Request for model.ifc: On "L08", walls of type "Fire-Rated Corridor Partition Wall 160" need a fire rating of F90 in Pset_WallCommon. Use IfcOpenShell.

First a look at what the model holds.

```python
import ifcopenshell
import ifcopenshell.util.element

model = ifcopenshell.open("model.ifc")
print(model.schema)
storey = next(s for s in model.by_type("IfcBuildingStorey") if s.Name == "L08")
walls = [e for e in ifcopenshell.util.element.get_decomposition(storey) if e.is_a("IfcWall")]
seen = {}
for e in walls:
    element_type = ifcopenshell.util.element.get_type(e)
    key = (element_type.Name if element_type != e and element_type else None, ifcopenshell.util.element.get_pset(e, "Pset_WallCommon", "FireRating"))
    seen[key] = seen.get(key, 0) + 1
for (name, value), count in sorted(seen.items(), key=str):
    print(count, "x", name, "|", value)
```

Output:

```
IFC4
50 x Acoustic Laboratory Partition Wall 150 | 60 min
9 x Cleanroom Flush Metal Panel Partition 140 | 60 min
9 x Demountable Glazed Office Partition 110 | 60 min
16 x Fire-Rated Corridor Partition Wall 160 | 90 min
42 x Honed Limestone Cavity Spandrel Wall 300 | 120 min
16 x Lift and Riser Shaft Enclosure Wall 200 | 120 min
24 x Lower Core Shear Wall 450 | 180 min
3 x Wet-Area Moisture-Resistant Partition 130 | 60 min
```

```python
import ifcopenshell
import ifcopenshell.api.pset
import ifcopenshell.util.element

model = ifcopenshell.open("model.ifc")

storey = next(s for s in model.by_type("IfcBuildingStorey") if s.Name == "L08")
walls = [e for e in ifcopenshell.util.element.get_decomposition(storey) if e.is_a("IfcWall")]

count = 0
for e in walls:
    element_type = ifcopenshell.util.element.get_type(e)
    if element_type in (None, e) or element_type.Name != "Fire-Rated Corridor Partition Wall 160":
        continue
    # add_pset returns the element's existing set when there is one.
    pset = ifcopenshell.api.pset.add_pset(model, product=e, name="Pset_WallCommon")
    ifcopenshell.api.pset.edit_pset(model, pset=pset, properties={"FireRating": "F90"})
    count += 1

print(count, "walls updated")

model.write("model_rev.ifc")
```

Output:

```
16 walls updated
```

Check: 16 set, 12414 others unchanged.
